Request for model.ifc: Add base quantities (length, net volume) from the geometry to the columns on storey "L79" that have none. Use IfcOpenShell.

First a look at what the model holds.

```python
import ifcopenshell
import ifcopenshell.util.element
import ifcopenshell.util.unit

model = ifcopenshell.open("model.ifc")
print(model.schema)
for unit_type in ("LENGTHUNIT", "AREAUNIT", "VOLUMEUNIT"):
    print(unit_type, ifcopenshell.util.unit.calculate_unit_scale(model, unit_type))
storey = next(s for s in model.by_type("IfcBuildingStorey") if s.Name == "L79")
columns = [e for e in ifcopenshell.util.element.get_decomposition(storey) if e.is_a("IfcColumn")]
for e in sorted(columns, key=lambda e: e.id()):
    print(e.id(), e.is_a(), e.Name, list(ifcopenshell.util.element.get_psets(e, qtos_only=True)), sep=" | ")
```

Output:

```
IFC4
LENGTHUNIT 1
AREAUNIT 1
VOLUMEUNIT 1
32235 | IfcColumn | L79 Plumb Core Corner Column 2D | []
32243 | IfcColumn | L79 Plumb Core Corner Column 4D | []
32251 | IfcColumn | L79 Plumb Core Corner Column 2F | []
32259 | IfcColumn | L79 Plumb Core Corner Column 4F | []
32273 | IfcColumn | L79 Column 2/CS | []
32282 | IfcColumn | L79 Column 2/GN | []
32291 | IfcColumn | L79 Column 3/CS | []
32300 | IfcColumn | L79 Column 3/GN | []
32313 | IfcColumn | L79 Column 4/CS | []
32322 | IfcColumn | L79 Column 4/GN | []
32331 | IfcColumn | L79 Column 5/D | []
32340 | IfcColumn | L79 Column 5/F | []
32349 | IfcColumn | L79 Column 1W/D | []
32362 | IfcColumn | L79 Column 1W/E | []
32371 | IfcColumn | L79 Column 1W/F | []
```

```python
import ifcopenshell
import ifcopenshell.api.pset
import ifcopenshell.geom
import ifcopenshell.util.element
import ifcopenshell.util.shape
import ifcopenshell.util.unit

model = ifcopenshell.open("model.ifc")
unit_scale = ifcopenshell.util.unit.calculate_unit_scale(model)
volume_scale = ifcopenshell.util.unit.calculate_unit_scale(model, "VOLUMEUNIT")
settings = ifcopenshell.geom.settings()

storey = next(s for s in model.by_type("IfcBuildingStorey") if s.Name == "L79")
columns = [e for e in ifcopenshell.util.element.get_decomposition(storey) if e.is_a("IfcColumn")]

for e in sorted(columns, key=lambda e: e.id()):
    if ifcopenshell.util.element.get_psets(e, qtos_only=True, should_inherit=False):
        continue
    # Geometry comes back in metres, in the element's own axes.
    shape = ifcopenshell.geom.create_shape(settings, e)
    values = {
        "Length": ifcopenshell.util.shape.get_z(shape.geometry) / unit_scale,
        "NetVolume": ifcopenshell.util.shape.get_volume(shape.geometry) / volume_scale,
    }
    qto = ifcopenshell.api.pset.add_qto(model, product=e, name="Qto_ColumnBaseQuantities")
    ifcopenshell.api.pset.edit_qto(model, qto=qto, properties=values)
    print(e.id(), {k: round(v, 3) for k, v in values.items()})

model.write("model_v2.ifc")
```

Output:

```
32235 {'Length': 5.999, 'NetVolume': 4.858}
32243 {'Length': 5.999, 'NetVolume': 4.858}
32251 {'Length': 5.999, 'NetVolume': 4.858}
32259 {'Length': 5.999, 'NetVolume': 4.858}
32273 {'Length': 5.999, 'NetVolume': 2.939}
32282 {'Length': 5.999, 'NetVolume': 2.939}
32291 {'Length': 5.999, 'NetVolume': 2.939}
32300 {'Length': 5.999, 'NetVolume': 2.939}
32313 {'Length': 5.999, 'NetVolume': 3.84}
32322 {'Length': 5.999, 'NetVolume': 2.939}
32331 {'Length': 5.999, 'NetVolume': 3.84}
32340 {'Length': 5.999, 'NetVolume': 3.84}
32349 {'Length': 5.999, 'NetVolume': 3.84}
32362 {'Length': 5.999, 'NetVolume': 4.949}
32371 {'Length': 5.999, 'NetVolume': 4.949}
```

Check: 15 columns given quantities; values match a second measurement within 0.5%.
